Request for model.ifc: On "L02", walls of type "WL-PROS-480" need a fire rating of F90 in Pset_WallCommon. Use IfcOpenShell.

First a look at what the model holds.

```python
import ifcopenshell
import ifcopenshell.util.element

model = ifcopenshell.open("model.ifc")
print(model.schema)
storey = next(s for s in model.by_type("IfcBuildingStorey") if s.Name == "L02")
walls = [e for e in ifcopenshell.util.element.get_decomposition(storey) if e.is_a("IfcWall")]
seen = {}
for e in walls:
    element_type = ifcopenshell.util.element.get_type(e)
    key = (element_type.Name if element_type != e and element_type else None, ifcopenshell.util.element.get_pset(e, "Pset_WallCommon", "FireRating"))
    seen[key] = seen.get(key, 0) + 1
for (name, value), count in sorted(seen.items(), key=str):
    print(count, "x", name, "|", value)
```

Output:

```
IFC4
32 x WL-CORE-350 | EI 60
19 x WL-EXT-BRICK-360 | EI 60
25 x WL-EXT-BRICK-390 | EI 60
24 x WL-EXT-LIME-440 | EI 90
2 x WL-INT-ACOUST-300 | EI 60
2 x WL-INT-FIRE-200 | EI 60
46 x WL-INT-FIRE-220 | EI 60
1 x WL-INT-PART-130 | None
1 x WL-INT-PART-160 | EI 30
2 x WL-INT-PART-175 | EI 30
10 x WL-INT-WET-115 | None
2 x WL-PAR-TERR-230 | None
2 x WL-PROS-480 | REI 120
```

```python
import ifcopenshell
import ifcopenshell.api.pset
import ifcopenshell.util.element

model = ifcopenshell.open("model.ifc")

storey = next(s for s in model.by_type("IfcBuildingStorey") if s.Name == "L02")
walls = [e for e in ifcopenshell.util.element.get_decomposition(storey) if e.is_a("IfcWall")]

count = 0
for e in walls:
    element_type = ifcopenshell.util.element.get_type(e)
    if element_type in (None, e) or element_type.Name != "WL-PROS-480":
        continue
    # add_pset returns the element's existing set when there is one.
    pset = ifcopenshell.api.pset.add_pset(model, product=e, name="Pset_WallCommon")
    ifcopenshell.api.pset.edit_pset(model, pset=pset, properties={"FireRating": "F90"})
    count += 1

print(count, "walls updated")

model.write("model_rev.ifc")
```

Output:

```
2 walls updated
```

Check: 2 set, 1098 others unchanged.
